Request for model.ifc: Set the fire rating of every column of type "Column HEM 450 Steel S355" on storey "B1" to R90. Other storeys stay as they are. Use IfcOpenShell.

First a look at what the model holds.

```python
import ifcopenshell
import ifcopenshell.util.element

model = ifcopenshell.open("model.ifc")
print(model.schema)
storey = next(s for s in model.by_type("IfcBuildingStorey") if s.Name == "B1")
columns = [e for e in ifcopenshell.util.element.get_decomposition(storey) if e.is_a("IfcColumn")]
seen = {}
for e in columns:
    element_type = ifcopenshell.util.element.get_type(e)
    key = (element_type.Name if element_type != e and element_type else None, ifcopenshell.util.element.get_pset(e, "Pset_ColumnCommon", "FireRating"))
    seen[key] = seen.get(key, 0) + 1
for (name, value), count in sorted(seen.items(), key=str):
    print(count, "x", name, "|", value)
```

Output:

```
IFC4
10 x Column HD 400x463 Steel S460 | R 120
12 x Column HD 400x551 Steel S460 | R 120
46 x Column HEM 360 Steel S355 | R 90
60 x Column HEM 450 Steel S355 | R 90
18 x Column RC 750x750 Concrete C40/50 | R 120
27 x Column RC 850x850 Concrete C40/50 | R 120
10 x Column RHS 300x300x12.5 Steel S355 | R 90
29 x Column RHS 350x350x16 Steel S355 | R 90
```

```python
import ifcopenshell
import ifcopenshell.api.pset
import ifcopenshell.util.element

model = ifcopenshell.open("model.ifc")

storey = next(s for s in model.by_type("IfcBuildingStorey") if s.Name == "B1")
columns = [e for e in ifcopenshell.util.element.get_decomposition(storey) if e.is_a("IfcColumn")]

count = 0
for e in columns:
    element_type = ifcopenshell.util.element.get_type(e)
    if element_type in (None, e) or element_type.Name != "Column HEM 450 Steel S355":
        continue
    # add_pset returns the element's existing set when there is one.
    pset = ifcopenshell.api.pset.add_pset(model, product=e, name="Pset_ColumnCommon")
    ifcopenshell.api.pset.edit_pset(model, pset=pset, properties={"FireRating": "R90"})
    count += 1

print(count, "columns updated")

model.write("model-out.ifc")
```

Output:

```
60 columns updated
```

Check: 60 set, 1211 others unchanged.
